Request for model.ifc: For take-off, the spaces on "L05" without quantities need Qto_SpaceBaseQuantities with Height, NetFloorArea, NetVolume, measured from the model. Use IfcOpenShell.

First a look at what the model holds.

```python
import ifcopenshell
import ifcopenshell.util.element
import ifcopenshell.util.unit

model = ifcopenshell.open("model.ifc")
print(model.schema)
for unit_type in ("LENGTHUNIT", "AREAUNIT", "VOLUMEUNIT"):
    print(unit_type, ifcopenshell.util.unit.calculate_unit_scale(model, unit_type))
storey = next(s for s in model.by_type("IfcBuildingStorey") if s.Name == "L05")
spaces = [e for e in ifcopenshell.util.element.get_decomposition(storey) if e.is_a("IfcSpace")]
for e in sorted(spaces, key=lambda e: e.id()):
    print(e.id(), e.is_a(), e.Name, list(ifcopenshell.util.element.get_psets(e, qtos_only=True)), sep=" | ")
```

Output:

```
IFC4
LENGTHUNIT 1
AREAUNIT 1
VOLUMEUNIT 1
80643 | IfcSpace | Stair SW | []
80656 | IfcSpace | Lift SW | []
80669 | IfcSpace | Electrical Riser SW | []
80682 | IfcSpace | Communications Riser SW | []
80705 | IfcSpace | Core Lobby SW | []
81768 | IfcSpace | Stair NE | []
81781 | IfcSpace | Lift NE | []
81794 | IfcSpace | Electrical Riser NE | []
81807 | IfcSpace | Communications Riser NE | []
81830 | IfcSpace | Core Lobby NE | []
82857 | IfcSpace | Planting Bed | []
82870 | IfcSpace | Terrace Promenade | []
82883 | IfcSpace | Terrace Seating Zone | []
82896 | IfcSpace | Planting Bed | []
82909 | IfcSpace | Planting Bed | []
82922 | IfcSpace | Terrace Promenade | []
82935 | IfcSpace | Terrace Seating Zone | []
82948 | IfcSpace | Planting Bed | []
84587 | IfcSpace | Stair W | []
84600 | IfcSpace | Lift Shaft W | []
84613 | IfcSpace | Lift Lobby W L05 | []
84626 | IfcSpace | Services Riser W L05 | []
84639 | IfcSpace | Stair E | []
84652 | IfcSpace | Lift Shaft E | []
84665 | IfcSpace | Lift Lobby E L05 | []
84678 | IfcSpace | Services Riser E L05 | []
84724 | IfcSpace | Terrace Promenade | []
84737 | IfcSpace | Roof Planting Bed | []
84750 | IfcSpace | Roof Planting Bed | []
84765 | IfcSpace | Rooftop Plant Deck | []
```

```python
import ifcopenshell
import ifcopenshell.api.pset
import ifcopenshell.geom
import ifcopenshell.util.element
import ifcopenshell.util.shape
import ifcopenshell.util.unit

model = ifcopenshell.open("model.ifc")
unit_scale = ifcopenshell.util.unit.calculate_unit_scale(model)
area_scale = ifcopenshell.util.unit.calculate_unit_scale(model, "AREAUNIT")
volume_scale = ifcopenshell.util.unit.calculate_unit_scale(model, "VOLUMEUNIT")
settings = ifcopenshell.geom.settings()

storey = next(s for s in model.by_type("IfcBuildingStorey") if s.Name == "L05")
spaces = [e for e in ifcopenshell.util.element.get_decomposition(storey) if e.is_a("IfcSpace")]

for e in sorted(spaces, key=lambda e: e.id()):
    if ifcopenshell.util.element.get_psets(e, qtos_only=True, should_inherit=False):
        continue
    # Geometry comes back in metres, in the element's own axes.
    shape = ifcopenshell.geom.create_shape(settings, e)
    values = {
        "Height": ifcopenshell.util.shape.get_z(shape.geometry) / unit_scale,
        "NetFloorArea": ifcopenshell.util.shape.get_footprint_area(shape.geometry) / area_scale,
        "NetVolume": ifcopenshell.util.shape.get_volume(shape.geometry) / volume_scale,
    }
    qto = ifcopenshell.api.pset.add_qto(model, product=e, name="Qto_SpaceBaseQuantities")
    ifcopenshell.api.pset.edit_qto(model, qto=qto, properties=values)
    print(e.id(), {k: round(v, 3) for k, v in values.items()})

model.write("model_rev.ifc")
```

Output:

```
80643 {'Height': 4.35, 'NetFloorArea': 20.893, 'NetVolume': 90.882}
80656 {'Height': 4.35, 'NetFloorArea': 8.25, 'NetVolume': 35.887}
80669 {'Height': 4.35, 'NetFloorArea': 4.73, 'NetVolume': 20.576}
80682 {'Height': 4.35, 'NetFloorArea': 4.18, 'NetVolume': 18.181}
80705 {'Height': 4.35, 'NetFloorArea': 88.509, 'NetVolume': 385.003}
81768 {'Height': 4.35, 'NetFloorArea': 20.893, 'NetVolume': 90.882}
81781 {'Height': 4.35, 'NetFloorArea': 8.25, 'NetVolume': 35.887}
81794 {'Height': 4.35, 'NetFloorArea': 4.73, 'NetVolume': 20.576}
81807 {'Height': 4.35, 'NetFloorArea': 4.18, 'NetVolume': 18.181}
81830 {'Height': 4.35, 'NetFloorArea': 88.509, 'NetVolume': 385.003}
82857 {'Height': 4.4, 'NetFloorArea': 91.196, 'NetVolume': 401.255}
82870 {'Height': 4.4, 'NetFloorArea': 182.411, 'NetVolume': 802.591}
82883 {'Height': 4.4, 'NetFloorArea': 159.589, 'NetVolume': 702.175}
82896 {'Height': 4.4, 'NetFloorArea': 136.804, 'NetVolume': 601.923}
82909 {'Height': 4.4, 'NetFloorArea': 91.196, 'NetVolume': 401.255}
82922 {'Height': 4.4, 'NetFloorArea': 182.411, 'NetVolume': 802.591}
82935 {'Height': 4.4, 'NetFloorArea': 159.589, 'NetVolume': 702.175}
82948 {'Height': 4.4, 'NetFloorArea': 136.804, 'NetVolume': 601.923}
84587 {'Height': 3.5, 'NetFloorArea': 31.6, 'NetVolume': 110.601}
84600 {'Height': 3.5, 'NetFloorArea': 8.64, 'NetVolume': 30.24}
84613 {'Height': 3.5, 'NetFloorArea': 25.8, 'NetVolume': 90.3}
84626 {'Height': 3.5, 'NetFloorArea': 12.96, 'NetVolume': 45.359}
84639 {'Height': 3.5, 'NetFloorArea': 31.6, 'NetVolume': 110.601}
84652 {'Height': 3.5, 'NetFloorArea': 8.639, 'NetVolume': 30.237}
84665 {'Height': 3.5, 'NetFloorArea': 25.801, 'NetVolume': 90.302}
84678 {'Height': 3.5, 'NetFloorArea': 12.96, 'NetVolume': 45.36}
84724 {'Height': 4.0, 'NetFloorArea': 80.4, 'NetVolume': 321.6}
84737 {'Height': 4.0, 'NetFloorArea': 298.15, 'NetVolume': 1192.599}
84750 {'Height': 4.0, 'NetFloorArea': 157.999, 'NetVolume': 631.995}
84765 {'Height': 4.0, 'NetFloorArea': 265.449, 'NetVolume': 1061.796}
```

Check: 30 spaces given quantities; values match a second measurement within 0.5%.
